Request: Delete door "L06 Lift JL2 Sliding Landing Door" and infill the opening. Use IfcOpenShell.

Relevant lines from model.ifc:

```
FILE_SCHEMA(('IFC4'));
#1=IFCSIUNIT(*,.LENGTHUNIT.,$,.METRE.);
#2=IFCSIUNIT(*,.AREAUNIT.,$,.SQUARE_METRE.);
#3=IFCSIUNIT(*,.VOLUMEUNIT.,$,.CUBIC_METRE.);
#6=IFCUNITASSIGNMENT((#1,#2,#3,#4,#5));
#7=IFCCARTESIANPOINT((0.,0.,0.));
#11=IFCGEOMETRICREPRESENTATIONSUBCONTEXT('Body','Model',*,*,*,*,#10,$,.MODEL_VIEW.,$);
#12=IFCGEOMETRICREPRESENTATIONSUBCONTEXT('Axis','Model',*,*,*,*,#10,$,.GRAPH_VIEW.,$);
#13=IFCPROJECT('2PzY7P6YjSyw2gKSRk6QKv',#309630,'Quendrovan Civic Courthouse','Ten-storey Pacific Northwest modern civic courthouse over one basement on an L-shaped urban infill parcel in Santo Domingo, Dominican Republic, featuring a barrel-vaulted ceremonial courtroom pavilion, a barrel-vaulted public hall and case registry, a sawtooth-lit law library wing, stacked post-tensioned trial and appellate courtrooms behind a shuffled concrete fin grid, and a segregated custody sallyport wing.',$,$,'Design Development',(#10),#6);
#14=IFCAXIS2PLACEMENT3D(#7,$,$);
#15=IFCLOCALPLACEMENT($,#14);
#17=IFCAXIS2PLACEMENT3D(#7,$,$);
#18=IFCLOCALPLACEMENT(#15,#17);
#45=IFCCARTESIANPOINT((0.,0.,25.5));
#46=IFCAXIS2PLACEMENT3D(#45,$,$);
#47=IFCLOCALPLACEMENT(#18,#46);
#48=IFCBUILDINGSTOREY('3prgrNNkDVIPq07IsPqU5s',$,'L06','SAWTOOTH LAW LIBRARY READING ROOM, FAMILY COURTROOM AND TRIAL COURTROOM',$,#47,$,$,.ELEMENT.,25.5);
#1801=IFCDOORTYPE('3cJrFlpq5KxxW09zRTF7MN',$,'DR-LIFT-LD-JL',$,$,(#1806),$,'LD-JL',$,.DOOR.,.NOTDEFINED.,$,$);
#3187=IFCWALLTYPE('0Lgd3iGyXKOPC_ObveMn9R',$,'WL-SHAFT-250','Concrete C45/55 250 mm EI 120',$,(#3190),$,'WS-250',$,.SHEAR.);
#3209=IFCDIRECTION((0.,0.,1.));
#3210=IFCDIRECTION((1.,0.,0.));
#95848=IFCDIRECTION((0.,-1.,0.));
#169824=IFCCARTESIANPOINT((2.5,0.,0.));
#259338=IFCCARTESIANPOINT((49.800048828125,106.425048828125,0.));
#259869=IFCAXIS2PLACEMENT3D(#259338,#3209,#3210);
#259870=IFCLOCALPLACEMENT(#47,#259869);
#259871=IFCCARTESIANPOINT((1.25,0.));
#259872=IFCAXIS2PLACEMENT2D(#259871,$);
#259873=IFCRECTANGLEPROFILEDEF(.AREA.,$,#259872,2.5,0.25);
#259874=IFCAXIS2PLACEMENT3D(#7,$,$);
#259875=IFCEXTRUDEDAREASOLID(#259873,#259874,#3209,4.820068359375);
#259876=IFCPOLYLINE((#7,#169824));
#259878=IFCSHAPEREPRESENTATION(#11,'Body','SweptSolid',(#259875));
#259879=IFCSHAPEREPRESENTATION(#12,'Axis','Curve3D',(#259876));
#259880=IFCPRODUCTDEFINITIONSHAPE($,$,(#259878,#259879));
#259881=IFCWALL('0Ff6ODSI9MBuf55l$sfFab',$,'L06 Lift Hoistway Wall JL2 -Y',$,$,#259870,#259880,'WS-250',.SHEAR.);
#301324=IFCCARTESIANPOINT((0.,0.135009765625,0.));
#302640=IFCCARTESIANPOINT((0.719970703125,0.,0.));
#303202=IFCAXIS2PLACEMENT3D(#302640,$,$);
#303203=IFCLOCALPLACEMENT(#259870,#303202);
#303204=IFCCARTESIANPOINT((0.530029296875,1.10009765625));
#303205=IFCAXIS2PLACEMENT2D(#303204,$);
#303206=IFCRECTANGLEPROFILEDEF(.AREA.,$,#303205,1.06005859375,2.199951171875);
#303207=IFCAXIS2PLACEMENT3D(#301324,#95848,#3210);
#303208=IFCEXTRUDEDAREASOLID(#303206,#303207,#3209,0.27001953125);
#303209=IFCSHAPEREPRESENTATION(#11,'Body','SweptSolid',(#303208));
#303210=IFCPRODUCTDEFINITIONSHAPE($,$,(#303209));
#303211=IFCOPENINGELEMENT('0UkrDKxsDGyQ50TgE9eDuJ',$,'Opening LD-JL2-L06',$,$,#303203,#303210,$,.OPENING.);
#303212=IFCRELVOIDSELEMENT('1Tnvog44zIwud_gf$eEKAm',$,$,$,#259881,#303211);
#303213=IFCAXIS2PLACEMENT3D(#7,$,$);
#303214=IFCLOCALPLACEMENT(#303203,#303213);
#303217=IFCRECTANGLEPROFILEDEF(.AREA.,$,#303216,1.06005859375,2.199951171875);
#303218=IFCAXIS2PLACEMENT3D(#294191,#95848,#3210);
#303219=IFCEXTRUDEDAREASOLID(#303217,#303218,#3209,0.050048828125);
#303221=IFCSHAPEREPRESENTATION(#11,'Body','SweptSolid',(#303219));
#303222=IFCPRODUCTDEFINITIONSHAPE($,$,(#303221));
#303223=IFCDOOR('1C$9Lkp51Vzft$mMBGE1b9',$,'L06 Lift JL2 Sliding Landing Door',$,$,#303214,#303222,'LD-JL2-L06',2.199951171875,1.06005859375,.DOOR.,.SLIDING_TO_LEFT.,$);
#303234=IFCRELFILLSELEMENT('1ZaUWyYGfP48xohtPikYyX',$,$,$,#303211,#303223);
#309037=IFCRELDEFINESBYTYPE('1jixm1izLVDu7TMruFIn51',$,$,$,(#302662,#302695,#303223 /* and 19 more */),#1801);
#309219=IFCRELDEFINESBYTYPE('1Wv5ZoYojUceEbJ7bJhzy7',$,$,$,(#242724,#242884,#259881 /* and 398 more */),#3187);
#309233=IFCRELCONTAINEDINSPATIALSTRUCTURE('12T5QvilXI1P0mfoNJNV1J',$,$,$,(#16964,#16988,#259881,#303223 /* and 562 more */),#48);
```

```python
import ifcopenshell
import ifcopenshell.api.feature
import ifcopenshell.api.root
import ifcopenshell.geom
import ifcopenshell.util.shape

model = ifcopenshell.open("model.ifc")
settings = ifcopenshell.geom.settings()


def volume(element):
    """Net volume in cubic metres, openings subtracted."""
    shape = ifcopenshell.geom.create_shape(settings, element)
    return ifcopenshell.util.shape.get_volume(shape.geometry)


door = model.by_guid("1C$9Lkp51Vzft$mMBGE1b9")
opening = door.FillsVoids[0].RelatingOpeningElement
wall = opening.VoidsElements[0].RelatingBuildingElement
before = volume(wall)

ifcopenshell.api.root.remove_product(model, product=door)
ifcopenshell.api.feature.remove_feature(model, feature=opening)

after = volume(wall)

print(f"wall volume {before:.3f} -> {after:.3f} m3")

model.write("model_rev.ifc")
```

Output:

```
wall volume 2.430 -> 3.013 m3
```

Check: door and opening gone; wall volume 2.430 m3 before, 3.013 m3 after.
